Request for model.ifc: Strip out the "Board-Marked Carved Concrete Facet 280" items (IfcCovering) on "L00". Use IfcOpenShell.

First a look at what the model holds.

```python
import ifcopenshell
import ifcopenshell.util.element

model = ifcopenshell.open("model.ifc")
print(model.schema)
storey = next(s for s in model.by_type("IfcBuildingStorey") if s.Name == "L00")
coverings = [e for e in ifcopenshell.util.element.get_decomposition(storey) if e.is_a("IfcCovering")]
seen = {}
for e in coverings:
    element_type = ifcopenshell.util.element.get_type(e)
    name = element_type.Name if element_type not in (None, e) else None
    seen[name] = seen.get(name, 0) + 1
for name, count in sorted(seen.items(), key=str):
    print(count, "x", name)
```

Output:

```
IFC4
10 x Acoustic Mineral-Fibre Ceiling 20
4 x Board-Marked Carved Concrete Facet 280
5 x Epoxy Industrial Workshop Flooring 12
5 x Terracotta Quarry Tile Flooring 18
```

```python
import ifcopenshell
import ifcopenshell.api.root
import ifcopenshell.util.element

model = ifcopenshell.open("model.ifc")

storey = next(s for s in model.by_type("IfcBuildingStorey") if s.Name == "L00")
coverings = [e for e in ifcopenshell.util.element.get_decomposition(storey) if e.is_a("IfcCovering")]
targets = [e for e in coverings if (t := ifcopenshell.util.element.get_type(e)) not in (None, e) and t.Name == "Board-Marked Carved Concrete Facet 280"]

for e in targets:
    ifcopenshell.api.root.remove_product(model, product=e)
print(len(targets), "removed")

model.write("model_v2.ifc")
```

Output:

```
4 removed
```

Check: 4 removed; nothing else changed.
